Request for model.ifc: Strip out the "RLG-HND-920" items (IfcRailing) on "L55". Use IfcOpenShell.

First a look at what the model holds.

```python
import ifcopenshell
import ifcopenshell.util.element

model = ifcopenshell.open("model.ifc")
print(model.schema)
storey = next(s for s in model.by_type("IfcBuildingStorey") if s.Name == "L55")
railings = [e for e in ifcopenshell.util.element.get_decomposition(storey) if e.is_a("IfcRailing")]
seen = {}
for e in railings:
    element_type = ifcopenshell.util.element.get_type(e)
    name = element_type.Name if element_type not in (None, e) else None
    seen[name] = seen.get(name, 0) + 1
for name, count in sorted(seen.items(), key=str):
    print(count, "x", name)
```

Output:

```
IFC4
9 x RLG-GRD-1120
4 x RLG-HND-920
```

```python
import ifcopenshell
import ifcopenshell.api.root
import ifcopenshell.util.element

model = ifcopenshell.open("model.ifc")

storey = next(s for s in model.by_type("IfcBuildingStorey") if s.Name == "L55")
railings = [e for e in ifcopenshell.util.element.get_decomposition(storey) if e.is_a("IfcRailing")]
targets = [e for e in railings if (t := ifcopenshell.util.element.get_type(e)) not in (None, e) and t.Name == "RLG-HND-920"]

for e in targets:
    ifcopenshell.api.root.remove_product(model, product=e)
print(len(targets), "removed")

model.write("model-out.ifc")
```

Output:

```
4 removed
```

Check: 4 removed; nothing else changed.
